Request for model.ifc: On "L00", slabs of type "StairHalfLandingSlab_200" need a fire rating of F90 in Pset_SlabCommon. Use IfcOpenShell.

First a look at what the model holds.

```python
import ifcopenshell
import ifcopenshell.util.element

model = ifcopenshell.open("model.ifc")
print(model.schema)
storey = next(s for s in model.by_type("IfcBuildingStorey") if s.Name == "L00")
slabs = [e for e in ifcopenshell.util.element.get_decomposition(storey) if e.is_a("IfcSlab")]
seen = {}
for e in slabs:
    element_type = ifcopenshell.util.element.get_type(e)
    key = (element_type.Name if element_type != e and element_type else None, ifcopenshell.util.element.get_pset(e, "Pset_SlabCommon", "FireRating"))
    seen[key] = seen.get(key, 0) + 1
for (name, value), count in sorted(seen.items(), key=str):
    print(count, "x", name, "|", value)
```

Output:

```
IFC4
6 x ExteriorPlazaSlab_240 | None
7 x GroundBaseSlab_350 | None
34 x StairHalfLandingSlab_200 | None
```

```python
import ifcopenshell
import ifcopenshell.api.pset
import ifcopenshell.util.element

model = ifcopenshell.open("model.ifc")

storey = next(s for s in model.by_type("IfcBuildingStorey") if s.Name == "L00")
slabs = [e for e in ifcopenshell.util.element.get_decomposition(storey) if e.is_a("IfcSlab")]

count = 0
for e in slabs:
    element_type = ifcopenshell.util.element.get_type(e)
    if element_type in (None, e) or element_type.Name != "StairHalfLandingSlab_200":
        continue
    # add_pset returns the element's existing set when there is one.
    pset = ifcopenshell.api.pset.add_pset(model, product=e, name="Pset_SlabCommon")
    ifcopenshell.api.pset.edit_pset(model, pset=pset, properties={"FireRating": "F90"})
    count += 1

print(count, "slabs updated")

model.write("model_v2.ifc")
```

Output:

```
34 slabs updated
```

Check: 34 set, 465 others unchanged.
